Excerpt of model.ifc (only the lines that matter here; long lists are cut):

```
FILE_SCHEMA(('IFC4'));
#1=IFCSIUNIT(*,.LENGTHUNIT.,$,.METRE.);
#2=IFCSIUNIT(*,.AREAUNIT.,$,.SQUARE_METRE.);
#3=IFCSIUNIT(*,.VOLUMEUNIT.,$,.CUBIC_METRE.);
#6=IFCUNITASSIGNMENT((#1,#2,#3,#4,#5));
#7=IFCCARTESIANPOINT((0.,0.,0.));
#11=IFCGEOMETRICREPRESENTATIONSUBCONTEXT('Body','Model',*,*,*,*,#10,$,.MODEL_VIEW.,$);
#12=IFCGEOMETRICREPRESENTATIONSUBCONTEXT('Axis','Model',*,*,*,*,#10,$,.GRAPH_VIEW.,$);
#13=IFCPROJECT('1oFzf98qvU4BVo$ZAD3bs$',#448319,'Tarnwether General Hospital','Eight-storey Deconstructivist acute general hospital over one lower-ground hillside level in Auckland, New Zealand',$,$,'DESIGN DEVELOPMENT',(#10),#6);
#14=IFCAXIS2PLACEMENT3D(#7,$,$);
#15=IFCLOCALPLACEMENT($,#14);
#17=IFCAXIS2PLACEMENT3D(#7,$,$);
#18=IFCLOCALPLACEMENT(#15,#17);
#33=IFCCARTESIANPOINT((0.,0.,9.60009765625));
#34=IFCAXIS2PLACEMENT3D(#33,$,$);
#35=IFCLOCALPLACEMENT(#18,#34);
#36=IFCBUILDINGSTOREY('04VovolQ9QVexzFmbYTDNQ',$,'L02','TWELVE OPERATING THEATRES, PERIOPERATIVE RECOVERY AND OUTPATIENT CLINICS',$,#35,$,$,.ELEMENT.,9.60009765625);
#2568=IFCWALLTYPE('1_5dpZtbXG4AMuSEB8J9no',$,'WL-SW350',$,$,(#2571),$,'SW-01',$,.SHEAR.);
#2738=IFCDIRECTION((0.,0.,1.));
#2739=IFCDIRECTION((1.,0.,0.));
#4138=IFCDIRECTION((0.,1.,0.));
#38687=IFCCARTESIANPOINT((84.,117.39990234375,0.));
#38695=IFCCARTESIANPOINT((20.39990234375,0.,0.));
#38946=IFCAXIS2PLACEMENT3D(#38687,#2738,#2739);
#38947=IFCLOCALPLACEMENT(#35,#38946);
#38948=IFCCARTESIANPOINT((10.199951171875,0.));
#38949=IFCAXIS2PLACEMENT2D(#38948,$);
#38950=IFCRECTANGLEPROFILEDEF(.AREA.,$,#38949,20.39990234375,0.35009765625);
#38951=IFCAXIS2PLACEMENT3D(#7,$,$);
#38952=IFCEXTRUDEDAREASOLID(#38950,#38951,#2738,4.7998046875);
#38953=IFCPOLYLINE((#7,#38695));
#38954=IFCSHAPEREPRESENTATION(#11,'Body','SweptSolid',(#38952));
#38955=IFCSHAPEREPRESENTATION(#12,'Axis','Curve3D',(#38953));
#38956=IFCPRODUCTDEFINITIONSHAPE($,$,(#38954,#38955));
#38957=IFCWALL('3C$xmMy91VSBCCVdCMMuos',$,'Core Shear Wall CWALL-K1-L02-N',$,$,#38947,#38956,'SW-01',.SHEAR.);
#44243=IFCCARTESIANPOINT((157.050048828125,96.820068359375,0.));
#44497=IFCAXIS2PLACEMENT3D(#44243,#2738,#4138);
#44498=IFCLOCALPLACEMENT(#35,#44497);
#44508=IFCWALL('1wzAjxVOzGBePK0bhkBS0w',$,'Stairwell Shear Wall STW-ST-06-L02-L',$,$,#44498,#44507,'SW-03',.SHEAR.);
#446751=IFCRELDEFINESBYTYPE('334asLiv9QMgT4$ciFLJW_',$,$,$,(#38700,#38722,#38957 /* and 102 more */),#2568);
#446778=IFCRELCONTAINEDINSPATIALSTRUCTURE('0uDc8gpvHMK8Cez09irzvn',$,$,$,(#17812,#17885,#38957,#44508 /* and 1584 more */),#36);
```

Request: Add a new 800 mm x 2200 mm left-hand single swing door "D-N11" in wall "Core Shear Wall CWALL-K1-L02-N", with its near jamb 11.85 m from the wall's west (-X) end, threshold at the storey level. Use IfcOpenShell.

```python
import numpy as np
import ifcopenshell
import ifcopenshell.api.feature
import ifcopenshell.api.geometry
import ifcopenshell.api.root
import ifcopenshell.api.spatial
import ifcopenshell.geom
import ifcopenshell.util.element
import ifcopenshell.util.placement
import ifcopenshell.util.representation
import ifcopenshell.util.shape
import ifcopenshell.util.unit

model = ifcopenshell.open("model.ifc")
unit_scale = ifcopenshell.util.unit.calculate_unit_scale(model)
settings = ifcopenshell.geom.settings()


def volume(element):
    """Net volume in cubic metres, openings subtracted."""
    shape = ifcopenshell.geom.create_shape(settings, element)
    return ifcopenshell.util.shape.get_volume(shape.geometry)


wall = model.by_guid("3C$xmMy91VSBCCVdCMMuos")
storey = ifcopenshell.util.element.get_container(wall, ifc_class="IfcBuildingStorey")
context = ifcopenshell.util.representation.get_context(model, "Model", "Body", "MODEL_VIEW")
before = volume(wall)

width, height, from_end, sill = 0.8, 2.2, 11.85, 0.0  # metres

# The wall runs along its own X axis, and the end named is its -X end.
wall_shape = ifcopenshell.geom.create_shape(settings, wall)
x, y, z = ifcopenshell.util.shape.get_vertices(wall_shape.geometry).T
start = x.min() + from_end
face, thickness = float(y.min()), float(y.max() - y.min())
wall_matrix = ifcopenshell.util.placement.get_local_placement(wall.ObjectPlacement)
level = ifcopenshell.util.placement.get_local_placement(storey.ObjectPlacement)[2, 3]


def in_wall(x, y):
    """Placement at x, y metres in the wall's axes, at sill height."""
    matrix = wall_matrix.copy()
    matrix[:, 3] = wall_matrix @ np.array([x / unit_scale, y / unit_scale, 0.0, 1.0])
    matrix[2, 3] = level + sill / unit_scale
    return matrix


# Opening: a box that overshoots both wall faces by 50 mm.
opening = ifcopenshell.api.root.create_entity(model, ifc_class="IfcOpeningElement", predefined_type="OPENING")
box = ifcopenshell.api.geometry.add_wall_representation(
    model, context=context, length=width, height=height, thickness=thickness + 0.1
)
ifcopenshell.api.geometry.assign_representation(model, product=opening, representation=box)
ifcopenshell.api.geometry.edit_object_placement(model, product=opening, matrix=in_wall(start, face - 0.05), is_si=False)
ifcopenshell.api.feature.add_feature(model, feature=opening, element=wall)

door = ifcopenshell.api.root.create_entity(model, ifc_class="IfcDoor", name="D-N11", predefined_type="DOOR")
door.OverallWidth, door.OverallHeight = width / unit_scale, height / unit_scale
door.OperationType = "SINGLE_SWING_LEFT"
body = ifcopenshell.api.geometry.add_door_representation(
    model,
    context=context,
    overall_width=door.OverallWidth,
    overall_height=door.OverallHeight,
    operation_type="SINGLE_SWING_LEFT",
    lining_properties={"LiningDepth": thickness / unit_scale, "ThresholdDepth": thickness / unit_scale},
)
ifcopenshell.api.geometry.assign_representation(model, product=door, representation=body)
ifcopenshell.api.spatial.assign_container(model, products=[door], relating_structure=storey)
ifcopenshell.api.feature.add_filling(model, opening=opening, element=door)

# The lining spans the wall, so the door starts at the wall face.
ifcopenshell.api.geometry.edit_object_placement(model, product=door, matrix=in_wall(start, face), is_si=False)

after = volume(wall)

print(f"wall volume {before:.3f} -> {after:.3f} m3")

model.write("model_rev.ifc")
```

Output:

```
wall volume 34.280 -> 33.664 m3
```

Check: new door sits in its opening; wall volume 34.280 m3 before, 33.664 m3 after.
